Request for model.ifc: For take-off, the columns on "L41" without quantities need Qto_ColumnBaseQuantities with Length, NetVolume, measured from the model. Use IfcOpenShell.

First a look at what the model holds.

```python
import ifcopenshell
import ifcopenshell.util.element
import ifcopenshell.util.unit

model = ifcopenshell.open("model.ifc")
print(model.schema)
for unit_type in ("LENGTHUNIT", "AREAUNIT", "VOLUMEUNIT"):
    print(unit_type, ifcopenshell.util.unit.calculate_unit_scale(model, unit_type))
storey = next(s for s in model.by_type("IfcBuildingStorey") if s.Name == "L41")
columns = [e for e in ifcopenshell.util.element.get_decomposition(storey) if e.is_a("IfcColumn")]
for e in sorted(columns, key=lambda e: e.id()):
    print(e.id(), e.is_a(), e.Name, list(ifcopenshell.util.element.get_psets(e, qtos_only=True)), sep=" | ")
```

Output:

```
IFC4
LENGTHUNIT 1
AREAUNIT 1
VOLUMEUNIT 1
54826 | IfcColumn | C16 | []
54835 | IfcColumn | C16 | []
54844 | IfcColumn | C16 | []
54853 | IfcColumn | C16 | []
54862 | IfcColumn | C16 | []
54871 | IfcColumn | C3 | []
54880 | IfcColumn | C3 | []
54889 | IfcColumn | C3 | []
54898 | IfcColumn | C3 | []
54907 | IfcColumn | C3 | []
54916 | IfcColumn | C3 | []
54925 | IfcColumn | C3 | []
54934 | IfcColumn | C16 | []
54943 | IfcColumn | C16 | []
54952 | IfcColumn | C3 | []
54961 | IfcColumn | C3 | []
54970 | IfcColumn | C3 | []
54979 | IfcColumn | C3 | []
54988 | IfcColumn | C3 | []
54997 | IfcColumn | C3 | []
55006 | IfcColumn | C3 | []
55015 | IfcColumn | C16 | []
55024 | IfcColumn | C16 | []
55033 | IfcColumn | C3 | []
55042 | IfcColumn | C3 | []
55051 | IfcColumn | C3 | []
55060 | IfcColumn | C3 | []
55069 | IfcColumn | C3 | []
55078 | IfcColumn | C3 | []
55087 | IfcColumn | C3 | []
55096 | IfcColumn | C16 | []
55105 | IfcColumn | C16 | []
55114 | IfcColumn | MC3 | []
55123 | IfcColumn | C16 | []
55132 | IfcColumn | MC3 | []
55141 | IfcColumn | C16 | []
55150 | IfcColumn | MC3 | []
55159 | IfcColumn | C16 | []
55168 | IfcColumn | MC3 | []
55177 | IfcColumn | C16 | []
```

```python
import ifcopenshell
import ifcopenshell.api.pset
import ifcopenshell.geom
import ifcopenshell.util.element
import ifcopenshell.util.shape
import ifcopenshell.util.unit

model = ifcopenshell.open("model.ifc")
unit_scale = ifcopenshell.util.unit.calculate_unit_scale(model)
volume_scale = ifcopenshell.util.unit.calculate_unit_scale(model, "VOLUMEUNIT")
settings = ifcopenshell.geom.settings()

storey = next(s for s in model.by_type("IfcBuildingStorey") if s.Name == "L41")
columns = [e for e in ifcopenshell.util.element.get_decomposition(storey) if e.is_a("IfcColumn")]

for e in sorted(columns, key=lambda e: e.id()):
    if ifcopenshell.util.element.get_psets(e, qtos_only=True, should_inherit=False):
        continue
    # Geometry comes back in metres, in the element's own axes.
    shape = ifcopenshell.geom.create_shape(settings, e)
    values = {
        "Length": ifcopenshell.util.shape.get_z(shape.geometry) / unit_scale,
        "NetVolume": ifcopenshell.util.shape.get_volume(shape.geometry) / volume_scale,
    }
    qto = ifcopenshell.api.pset.add_qto(model, product=e, name="Qto_ColumnBaseQuantities")
    ifcopenshell.api.pset.edit_qto(model, qto=qto, properties=values)
    print(e.id(), {k: round(v, 3) for k, v in values.items()})

model.write("model_v2.ifc")
```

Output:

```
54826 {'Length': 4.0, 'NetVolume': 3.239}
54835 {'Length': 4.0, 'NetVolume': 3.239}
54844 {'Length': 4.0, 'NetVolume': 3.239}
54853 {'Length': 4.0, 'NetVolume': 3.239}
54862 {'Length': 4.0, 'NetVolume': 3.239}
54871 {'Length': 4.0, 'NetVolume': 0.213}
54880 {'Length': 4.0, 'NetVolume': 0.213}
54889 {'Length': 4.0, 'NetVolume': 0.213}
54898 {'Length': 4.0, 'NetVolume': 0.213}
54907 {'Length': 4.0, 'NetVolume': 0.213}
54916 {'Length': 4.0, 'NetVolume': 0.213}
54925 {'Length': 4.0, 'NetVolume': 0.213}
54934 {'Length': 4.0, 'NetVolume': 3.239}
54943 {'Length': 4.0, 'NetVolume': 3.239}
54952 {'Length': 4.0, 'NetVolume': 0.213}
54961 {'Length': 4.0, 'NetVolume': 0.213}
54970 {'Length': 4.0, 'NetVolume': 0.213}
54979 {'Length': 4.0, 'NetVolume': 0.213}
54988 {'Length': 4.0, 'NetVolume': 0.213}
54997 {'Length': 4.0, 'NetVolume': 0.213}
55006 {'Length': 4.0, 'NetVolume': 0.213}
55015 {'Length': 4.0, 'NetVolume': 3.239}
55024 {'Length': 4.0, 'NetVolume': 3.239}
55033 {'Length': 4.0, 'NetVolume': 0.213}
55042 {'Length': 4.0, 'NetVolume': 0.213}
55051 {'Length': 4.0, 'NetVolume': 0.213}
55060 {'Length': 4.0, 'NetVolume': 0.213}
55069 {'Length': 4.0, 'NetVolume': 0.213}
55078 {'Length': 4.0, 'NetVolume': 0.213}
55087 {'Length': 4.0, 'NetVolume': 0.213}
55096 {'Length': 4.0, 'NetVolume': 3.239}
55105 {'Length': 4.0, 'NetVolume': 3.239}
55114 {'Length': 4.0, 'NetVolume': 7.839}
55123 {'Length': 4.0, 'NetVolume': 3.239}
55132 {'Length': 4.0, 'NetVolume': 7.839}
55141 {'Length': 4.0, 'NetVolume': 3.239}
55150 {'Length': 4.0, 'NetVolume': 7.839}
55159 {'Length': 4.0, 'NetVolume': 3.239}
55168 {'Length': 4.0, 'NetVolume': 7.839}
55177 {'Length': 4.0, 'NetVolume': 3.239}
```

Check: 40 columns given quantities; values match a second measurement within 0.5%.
